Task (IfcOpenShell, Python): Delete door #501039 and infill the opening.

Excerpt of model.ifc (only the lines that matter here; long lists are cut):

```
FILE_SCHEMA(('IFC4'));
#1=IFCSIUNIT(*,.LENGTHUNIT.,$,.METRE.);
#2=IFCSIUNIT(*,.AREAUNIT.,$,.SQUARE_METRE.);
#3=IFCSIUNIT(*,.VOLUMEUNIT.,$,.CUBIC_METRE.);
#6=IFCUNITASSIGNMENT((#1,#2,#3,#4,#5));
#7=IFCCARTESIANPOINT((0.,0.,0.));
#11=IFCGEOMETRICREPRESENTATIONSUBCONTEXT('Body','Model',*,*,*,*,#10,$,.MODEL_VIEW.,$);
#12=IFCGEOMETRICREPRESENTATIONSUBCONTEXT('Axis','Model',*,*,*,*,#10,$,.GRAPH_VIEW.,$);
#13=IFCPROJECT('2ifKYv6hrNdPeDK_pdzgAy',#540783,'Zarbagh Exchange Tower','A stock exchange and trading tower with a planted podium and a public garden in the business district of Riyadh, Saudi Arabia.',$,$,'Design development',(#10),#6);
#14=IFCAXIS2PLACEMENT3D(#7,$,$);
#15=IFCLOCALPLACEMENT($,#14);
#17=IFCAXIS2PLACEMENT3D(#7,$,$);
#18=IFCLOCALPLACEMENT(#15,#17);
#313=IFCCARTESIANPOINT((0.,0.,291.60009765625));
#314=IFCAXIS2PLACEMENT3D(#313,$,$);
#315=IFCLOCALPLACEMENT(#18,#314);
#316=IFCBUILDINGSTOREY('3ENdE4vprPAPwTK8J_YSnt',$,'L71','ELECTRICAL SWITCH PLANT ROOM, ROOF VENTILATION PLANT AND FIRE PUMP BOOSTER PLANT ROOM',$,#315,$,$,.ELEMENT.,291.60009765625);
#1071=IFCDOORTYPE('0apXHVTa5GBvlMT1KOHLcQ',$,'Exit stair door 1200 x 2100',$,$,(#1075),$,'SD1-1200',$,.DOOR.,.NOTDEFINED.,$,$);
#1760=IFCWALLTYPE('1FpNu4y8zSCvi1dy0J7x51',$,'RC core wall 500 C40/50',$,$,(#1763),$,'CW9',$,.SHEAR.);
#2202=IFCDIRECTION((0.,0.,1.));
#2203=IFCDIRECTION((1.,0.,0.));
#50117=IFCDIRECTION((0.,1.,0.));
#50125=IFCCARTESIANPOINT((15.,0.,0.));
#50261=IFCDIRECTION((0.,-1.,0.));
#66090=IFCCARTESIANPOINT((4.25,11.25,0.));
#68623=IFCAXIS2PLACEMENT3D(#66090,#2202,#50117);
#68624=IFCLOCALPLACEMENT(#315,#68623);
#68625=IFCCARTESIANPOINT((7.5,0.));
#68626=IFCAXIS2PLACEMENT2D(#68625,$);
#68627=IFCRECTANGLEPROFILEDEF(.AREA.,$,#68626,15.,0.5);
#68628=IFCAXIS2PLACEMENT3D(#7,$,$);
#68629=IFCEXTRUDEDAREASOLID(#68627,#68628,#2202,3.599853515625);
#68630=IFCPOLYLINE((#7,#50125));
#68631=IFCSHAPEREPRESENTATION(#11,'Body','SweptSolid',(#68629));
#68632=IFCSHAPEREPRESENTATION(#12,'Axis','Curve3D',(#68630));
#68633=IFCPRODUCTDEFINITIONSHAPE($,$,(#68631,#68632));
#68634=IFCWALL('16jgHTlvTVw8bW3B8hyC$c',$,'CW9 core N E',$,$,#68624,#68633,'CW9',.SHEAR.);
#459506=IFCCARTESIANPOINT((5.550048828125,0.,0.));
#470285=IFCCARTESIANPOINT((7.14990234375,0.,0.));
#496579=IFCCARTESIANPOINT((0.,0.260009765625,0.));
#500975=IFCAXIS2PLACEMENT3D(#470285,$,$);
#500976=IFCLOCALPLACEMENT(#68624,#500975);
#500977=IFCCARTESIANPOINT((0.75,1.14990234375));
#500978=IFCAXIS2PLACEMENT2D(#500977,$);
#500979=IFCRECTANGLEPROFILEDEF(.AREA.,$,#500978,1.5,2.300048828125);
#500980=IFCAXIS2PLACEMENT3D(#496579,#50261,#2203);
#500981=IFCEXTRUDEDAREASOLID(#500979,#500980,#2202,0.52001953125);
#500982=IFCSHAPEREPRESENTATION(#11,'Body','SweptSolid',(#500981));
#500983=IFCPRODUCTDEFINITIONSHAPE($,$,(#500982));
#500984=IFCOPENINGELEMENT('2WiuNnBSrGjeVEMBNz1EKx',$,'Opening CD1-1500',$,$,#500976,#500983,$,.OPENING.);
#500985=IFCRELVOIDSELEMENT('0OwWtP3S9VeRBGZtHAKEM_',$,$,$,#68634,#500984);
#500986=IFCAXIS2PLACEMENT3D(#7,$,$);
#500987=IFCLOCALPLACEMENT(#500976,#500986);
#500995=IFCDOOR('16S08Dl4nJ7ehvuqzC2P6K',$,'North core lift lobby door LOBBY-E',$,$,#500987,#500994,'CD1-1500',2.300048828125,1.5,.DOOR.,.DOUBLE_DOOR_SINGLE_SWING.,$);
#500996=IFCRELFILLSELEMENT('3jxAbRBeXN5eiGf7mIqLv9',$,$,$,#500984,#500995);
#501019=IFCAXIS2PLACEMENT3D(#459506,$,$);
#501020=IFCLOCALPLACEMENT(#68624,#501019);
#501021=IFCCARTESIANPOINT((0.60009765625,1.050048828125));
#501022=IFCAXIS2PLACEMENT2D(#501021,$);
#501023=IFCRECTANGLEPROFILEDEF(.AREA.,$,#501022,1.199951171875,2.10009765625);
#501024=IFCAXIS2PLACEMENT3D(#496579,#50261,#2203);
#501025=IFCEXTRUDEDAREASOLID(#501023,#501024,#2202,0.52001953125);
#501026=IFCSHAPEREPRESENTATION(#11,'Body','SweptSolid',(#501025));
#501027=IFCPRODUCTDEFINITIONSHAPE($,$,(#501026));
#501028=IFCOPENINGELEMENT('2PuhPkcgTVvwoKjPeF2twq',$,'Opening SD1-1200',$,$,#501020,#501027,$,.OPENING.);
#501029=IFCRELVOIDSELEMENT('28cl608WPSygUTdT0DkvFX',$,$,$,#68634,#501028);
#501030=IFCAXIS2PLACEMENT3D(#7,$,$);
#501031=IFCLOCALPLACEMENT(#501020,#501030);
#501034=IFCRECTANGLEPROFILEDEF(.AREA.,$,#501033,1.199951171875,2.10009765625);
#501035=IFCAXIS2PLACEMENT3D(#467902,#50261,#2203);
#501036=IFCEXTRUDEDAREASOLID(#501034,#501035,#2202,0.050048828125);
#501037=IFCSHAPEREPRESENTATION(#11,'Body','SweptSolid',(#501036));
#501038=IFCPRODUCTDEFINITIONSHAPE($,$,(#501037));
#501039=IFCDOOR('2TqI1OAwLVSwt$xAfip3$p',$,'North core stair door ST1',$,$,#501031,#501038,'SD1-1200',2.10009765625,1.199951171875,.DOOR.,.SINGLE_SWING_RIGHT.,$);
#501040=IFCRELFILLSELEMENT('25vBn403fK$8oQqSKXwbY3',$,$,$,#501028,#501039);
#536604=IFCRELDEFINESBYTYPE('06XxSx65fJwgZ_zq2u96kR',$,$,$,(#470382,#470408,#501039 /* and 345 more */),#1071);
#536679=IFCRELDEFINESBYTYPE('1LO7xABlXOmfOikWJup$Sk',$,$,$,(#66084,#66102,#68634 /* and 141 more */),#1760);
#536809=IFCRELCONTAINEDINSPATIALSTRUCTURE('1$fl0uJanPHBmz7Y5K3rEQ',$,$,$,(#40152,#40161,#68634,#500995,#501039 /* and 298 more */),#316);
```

```python
import ifcopenshell
import ifcopenshell.api.feature
import ifcopenshell.api.root
import ifcopenshell.geom
import ifcopenshell.util.shape

model = ifcopenshell.open("model.ifc")
settings = ifcopenshell.geom.settings()


def volume(element):
    """Net volume in cubic metres, openings subtracted."""
    shape = ifcopenshell.geom.create_shape(settings, element)
    return ifcopenshell.util.shape.get_volume(shape.geometry)


door = model.by_guid("2TqI1OAwLVSwt$xAfip3$p")
opening = door.FillsVoids[0].RelatingOpeningElement
wall = opening.VoidsElements[0].RelatingBuildingElement
before = volume(wall)

ifcopenshell.api.root.remove_product(model, product=door)
ifcopenshell.api.feature.remove_feature(model, feature=opening)

after = volume(wall)

print(f"wall volume {before:.3f} -> {after:.3f} m3")

model.write("model_rev.ifc")
```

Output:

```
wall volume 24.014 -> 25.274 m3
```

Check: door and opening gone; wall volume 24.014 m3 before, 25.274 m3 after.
